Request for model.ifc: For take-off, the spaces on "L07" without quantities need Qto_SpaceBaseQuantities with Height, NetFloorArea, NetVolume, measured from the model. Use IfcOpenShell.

First a look at what the model holds.

```python
import ifcopenshell
import ifcopenshell.util.element
import ifcopenshell.util.unit

model = ifcopenshell.open("model.ifc")
print(model.schema)
for unit_type in ("LENGTHUNIT", "AREAUNIT", "VOLUMEUNIT"):
    print(unit_type, ifcopenshell.util.unit.calculate_unit_scale(model, unit_type))
storey = next(s for s in model.by_type("IfcBuildingStorey") if s.Name == "L07")
spaces = [e for e in ifcopenshell.util.element.get_decomposition(storey) if e.is_a("IfcSpace")]
for e in sorted(spaces, key=lambda e: e.id()):
    print(e.id(), e.is_a(), e.Name, list(ifcopenshell.util.element.get_psets(e, qtos_only=True)), sep=" | ")
```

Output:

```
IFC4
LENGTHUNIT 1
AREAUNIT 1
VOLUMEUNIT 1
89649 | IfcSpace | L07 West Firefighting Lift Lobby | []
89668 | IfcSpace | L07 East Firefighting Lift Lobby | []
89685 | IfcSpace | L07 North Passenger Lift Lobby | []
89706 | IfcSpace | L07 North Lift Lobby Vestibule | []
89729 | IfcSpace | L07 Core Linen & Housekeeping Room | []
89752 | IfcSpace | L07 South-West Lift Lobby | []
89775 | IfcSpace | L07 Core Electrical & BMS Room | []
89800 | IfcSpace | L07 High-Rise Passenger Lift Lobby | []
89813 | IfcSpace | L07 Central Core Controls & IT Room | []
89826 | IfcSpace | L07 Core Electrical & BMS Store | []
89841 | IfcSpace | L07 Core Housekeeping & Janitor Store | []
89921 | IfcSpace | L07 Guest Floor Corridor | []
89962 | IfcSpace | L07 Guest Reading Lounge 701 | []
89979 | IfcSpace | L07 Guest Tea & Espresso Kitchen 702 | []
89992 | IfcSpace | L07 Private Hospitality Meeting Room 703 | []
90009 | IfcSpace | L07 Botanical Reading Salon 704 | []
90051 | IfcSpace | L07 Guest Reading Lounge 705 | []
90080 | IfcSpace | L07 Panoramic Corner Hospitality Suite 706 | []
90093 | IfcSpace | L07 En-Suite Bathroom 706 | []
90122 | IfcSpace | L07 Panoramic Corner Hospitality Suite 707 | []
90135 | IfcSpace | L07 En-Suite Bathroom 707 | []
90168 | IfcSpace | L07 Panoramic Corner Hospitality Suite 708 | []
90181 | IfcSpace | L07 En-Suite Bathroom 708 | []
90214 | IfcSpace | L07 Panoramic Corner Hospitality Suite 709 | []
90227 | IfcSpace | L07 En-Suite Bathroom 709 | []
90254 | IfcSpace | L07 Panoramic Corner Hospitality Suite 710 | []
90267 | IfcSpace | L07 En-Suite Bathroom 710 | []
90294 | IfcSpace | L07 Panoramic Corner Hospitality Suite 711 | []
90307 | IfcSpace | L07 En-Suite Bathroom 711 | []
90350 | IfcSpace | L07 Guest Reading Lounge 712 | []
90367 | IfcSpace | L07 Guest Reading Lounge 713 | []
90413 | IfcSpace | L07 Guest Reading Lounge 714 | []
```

```python
import ifcopenshell
import ifcopenshell.api.pset
import ifcopenshell.geom
import ifcopenshell.util.element
import ifcopenshell.util.shape
import ifcopenshell.util.unit

model = ifcopenshell.open("model.ifc")
unit_scale = ifcopenshell.util.unit.calculate_unit_scale(model)
area_scale = ifcopenshell.util.unit.calculate_unit_scale(model, "AREAUNIT")
volume_scale = ifcopenshell.util.unit.calculate_unit_scale(model, "VOLUMEUNIT")
settings = ifcopenshell.geom.settings()

storey = next(s for s in model.by_type("IfcBuildingStorey") if s.Name == "L07")
spaces = [e for e in ifcopenshell.util.element.get_decomposition(storey) if e.is_a("IfcSpace")]

for e in sorted(spaces, key=lambda e: e.id()):
    if ifcopenshell.util.element.get_psets(e, qtos_only=True, should_inherit=False):
        continue
    # Geometry comes back in metres, in the element's own axes.
    shape = ifcopenshell.geom.create_shape(settings, e)
    values = {
        "Height": ifcopenshell.util.shape.get_z(shape.geometry) / unit_scale,
        "NetFloorArea": ifcopenshell.util.shape.get_footprint_area(shape.geometry) / area_scale,
        "NetVolume": ifcopenshell.util.shape.get_volume(shape.geometry) / volume_scale,
    }
    qto = ifcopenshell.api.pset.add_qto(model, product=e, name="Qto_SpaceBaseQuantities")
    ifcopenshell.api.pset.edit_qto(model, qto=qto, properties=values)
    print(e.id(), {k: round(v, 3) for k, v in values.items()})

model.write("model_v2.ifc")
```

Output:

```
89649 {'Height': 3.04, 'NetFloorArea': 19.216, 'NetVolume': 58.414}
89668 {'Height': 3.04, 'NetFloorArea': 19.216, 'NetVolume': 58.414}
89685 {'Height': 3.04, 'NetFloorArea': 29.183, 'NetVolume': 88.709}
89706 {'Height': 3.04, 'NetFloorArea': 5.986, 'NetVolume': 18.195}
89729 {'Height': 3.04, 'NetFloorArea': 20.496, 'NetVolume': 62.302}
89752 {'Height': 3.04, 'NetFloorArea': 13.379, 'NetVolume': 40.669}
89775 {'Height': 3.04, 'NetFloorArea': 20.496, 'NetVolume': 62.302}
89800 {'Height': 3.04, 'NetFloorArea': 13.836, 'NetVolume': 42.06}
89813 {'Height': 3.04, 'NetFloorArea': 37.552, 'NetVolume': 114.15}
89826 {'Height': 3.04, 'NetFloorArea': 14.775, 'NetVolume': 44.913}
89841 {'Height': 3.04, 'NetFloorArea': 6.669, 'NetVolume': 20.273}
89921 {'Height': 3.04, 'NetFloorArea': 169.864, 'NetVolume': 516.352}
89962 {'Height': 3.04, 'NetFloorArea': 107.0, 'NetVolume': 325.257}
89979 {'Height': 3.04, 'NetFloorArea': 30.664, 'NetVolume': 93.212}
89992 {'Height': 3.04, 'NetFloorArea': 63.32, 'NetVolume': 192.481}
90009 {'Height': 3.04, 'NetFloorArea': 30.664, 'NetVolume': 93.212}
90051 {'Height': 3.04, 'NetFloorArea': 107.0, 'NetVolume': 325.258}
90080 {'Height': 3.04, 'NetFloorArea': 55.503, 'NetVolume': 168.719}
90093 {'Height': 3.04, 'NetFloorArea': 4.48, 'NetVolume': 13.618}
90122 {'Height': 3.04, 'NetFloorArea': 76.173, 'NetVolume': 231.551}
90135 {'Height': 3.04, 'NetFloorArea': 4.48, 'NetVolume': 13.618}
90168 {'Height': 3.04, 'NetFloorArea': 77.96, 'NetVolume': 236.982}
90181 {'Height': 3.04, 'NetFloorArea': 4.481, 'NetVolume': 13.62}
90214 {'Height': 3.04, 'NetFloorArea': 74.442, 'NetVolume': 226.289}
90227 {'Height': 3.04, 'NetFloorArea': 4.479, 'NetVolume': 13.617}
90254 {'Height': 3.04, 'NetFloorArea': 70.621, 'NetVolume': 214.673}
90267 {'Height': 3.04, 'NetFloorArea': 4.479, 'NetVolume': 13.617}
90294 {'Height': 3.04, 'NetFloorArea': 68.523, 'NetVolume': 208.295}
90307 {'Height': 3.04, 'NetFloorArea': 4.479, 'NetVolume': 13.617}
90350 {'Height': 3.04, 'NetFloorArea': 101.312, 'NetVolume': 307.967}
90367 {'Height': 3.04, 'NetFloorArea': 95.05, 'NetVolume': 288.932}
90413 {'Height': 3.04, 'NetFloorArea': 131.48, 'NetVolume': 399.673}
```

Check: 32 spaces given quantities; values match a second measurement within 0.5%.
